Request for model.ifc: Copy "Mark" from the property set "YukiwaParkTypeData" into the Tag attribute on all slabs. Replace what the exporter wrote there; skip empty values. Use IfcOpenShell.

First a look at what the model holds.

```python
import ifcopenshell
import ifcopenshell.util.element

model = ifcopenshell.open("model.ifc")
print(model.schema)
slabs = model.by_type("IfcSlab")
print(len(slabs), "slabs")
for e in slabs[:8]:
    source = ifcopenshell.util.element.get_pset(e, "YukiwaParkTypeData", "Mark")
    target = e.Tag
    print(e.id(), repr(source), repr(target), sep=" | ")
```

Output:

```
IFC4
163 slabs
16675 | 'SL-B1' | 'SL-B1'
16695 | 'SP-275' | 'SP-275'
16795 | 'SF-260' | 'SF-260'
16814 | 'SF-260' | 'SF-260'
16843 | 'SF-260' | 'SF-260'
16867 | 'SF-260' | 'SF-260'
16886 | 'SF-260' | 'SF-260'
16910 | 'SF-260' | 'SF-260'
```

```python
import ifcopenshell
import ifcopenshell.util.element

model = ifcopenshell.open("model.ifc")

count = 0
for e in model.by_type("IfcSlab"):
    value = ifcopenshell.util.element.get_pset(e, "YukiwaParkTypeData", "Mark")
    current = e.Tag
    if not value or not value.strip() or current == value:
        continue
    e.Tag = value
    count += 1

print(count, "slabs updated")

model.write("model_updated.ifc")
```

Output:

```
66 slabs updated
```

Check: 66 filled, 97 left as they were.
